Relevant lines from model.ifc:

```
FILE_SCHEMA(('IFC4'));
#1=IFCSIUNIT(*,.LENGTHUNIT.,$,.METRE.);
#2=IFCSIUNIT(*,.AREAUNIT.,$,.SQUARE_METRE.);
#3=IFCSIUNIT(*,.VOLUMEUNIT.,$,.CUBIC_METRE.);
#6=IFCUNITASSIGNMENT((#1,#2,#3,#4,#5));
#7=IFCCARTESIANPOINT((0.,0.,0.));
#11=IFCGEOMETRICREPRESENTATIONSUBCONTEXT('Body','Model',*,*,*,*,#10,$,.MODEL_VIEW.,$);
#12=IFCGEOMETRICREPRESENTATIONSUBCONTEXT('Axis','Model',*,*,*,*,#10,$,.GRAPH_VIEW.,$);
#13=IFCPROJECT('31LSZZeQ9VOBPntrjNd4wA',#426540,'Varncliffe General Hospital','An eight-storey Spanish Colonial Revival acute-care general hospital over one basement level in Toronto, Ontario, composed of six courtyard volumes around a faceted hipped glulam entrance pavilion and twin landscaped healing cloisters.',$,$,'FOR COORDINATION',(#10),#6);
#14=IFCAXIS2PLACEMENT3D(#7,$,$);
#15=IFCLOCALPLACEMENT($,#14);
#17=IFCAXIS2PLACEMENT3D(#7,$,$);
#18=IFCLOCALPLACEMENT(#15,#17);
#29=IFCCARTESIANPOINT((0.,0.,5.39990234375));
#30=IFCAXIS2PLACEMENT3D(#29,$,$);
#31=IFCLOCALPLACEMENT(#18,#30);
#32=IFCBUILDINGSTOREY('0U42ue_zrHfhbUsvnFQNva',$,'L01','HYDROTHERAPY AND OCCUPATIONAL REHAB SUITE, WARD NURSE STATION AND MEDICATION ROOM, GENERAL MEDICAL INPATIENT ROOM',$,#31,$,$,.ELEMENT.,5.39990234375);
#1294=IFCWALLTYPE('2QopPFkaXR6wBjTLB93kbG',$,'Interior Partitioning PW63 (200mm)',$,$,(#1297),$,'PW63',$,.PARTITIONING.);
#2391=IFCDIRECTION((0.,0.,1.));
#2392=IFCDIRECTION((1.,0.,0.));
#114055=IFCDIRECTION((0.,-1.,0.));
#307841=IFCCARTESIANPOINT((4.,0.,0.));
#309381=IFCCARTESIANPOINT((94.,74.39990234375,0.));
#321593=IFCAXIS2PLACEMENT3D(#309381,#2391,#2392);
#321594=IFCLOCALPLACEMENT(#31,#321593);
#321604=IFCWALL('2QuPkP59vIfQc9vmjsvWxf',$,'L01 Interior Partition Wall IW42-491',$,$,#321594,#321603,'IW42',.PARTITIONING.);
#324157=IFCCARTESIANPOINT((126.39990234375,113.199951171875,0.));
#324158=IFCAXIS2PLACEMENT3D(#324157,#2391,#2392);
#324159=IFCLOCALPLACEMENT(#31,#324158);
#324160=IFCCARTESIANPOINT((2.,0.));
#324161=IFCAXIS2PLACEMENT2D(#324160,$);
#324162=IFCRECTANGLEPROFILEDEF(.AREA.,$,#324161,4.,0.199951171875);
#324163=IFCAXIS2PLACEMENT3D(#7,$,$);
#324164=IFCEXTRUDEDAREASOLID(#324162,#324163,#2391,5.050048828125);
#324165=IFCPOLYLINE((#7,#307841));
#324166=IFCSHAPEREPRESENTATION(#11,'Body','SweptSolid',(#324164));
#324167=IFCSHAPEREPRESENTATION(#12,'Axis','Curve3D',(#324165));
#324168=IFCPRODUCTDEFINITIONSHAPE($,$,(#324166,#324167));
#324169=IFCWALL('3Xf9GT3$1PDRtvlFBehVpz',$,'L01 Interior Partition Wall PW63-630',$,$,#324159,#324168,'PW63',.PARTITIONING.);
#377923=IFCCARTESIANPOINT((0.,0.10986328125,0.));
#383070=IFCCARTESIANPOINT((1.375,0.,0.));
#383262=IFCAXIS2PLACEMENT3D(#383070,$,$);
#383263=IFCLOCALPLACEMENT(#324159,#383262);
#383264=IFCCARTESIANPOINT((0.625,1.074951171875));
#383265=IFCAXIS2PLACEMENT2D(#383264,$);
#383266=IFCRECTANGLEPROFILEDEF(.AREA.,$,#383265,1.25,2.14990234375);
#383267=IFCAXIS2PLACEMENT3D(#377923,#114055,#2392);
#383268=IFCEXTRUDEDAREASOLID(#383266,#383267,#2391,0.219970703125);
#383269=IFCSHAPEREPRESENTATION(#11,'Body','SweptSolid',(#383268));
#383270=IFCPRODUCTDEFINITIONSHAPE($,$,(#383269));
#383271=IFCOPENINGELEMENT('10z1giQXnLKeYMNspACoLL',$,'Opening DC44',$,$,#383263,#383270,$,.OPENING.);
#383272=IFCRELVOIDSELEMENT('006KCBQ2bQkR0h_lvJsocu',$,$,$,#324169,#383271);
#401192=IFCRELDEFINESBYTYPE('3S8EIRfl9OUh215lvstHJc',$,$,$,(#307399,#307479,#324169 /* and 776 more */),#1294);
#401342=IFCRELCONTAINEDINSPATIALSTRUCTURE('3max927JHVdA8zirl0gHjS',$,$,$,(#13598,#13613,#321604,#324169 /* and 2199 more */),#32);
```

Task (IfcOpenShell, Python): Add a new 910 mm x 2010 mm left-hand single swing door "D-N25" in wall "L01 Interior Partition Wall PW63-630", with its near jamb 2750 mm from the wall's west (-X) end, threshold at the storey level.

```python
import numpy as np
import ifcopenshell
import ifcopenshell.api.feature
import ifcopenshell.api.geometry
import ifcopenshell.api.root
import ifcopenshell.api.spatial
import ifcopenshell.geom
import ifcopenshell.util.element
import ifcopenshell.util.placement
import ifcopenshell.util.representation
import ifcopenshell.util.shape
import ifcopenshell.util.unit

model = ifcopenshell.open("model.ifc")
unit_scale = ifcopenshell.util.unit.calculate_unit_scale(model)
settings = ifcopenshell.geom.settings()


def volume(element):
    """Net volume in cubic metres, openings subtracted."""
    shape = ifcopenshell.geom.create_shape(settings, element)
    return ifcopenshell.util.shape.get_volume(shape.geometry)


wall = model.by_guid("3Xf9GT3$1PDRtvlFBehVpz")
storey = ifcopenshell.util.element.get_container(wall, ifc_class="IfcBuildingStorey")
context = ifcopenshell.util.representation.get_context(model, "Model", "Body", "MODEL_VIEW")
before = volume(wall)

width, height, from_end, sill = 0.91, 2.01, 2.75, 0.0  # metres

# The wall runs along its own X axis, and the end named is its -X end.
wall_shape = ifcopenshell.geom.create_shape(settings, wall)
x, y, z = ifcopenshell.util.shape.get_vertices(wall_shape.geometry).T
start = x.min() + from_end
face, thickness = float(y.min()), float(y.max() - y.min())
wall_matrix = ifcopenshell.util.placement.get_local_placement(wall.ObjectPlacement)
level = ifcopenshell.util.placement.get_local_placement(storey.ObjectPlacement)[2, 3]


def in_wall(x, y):
    """Placement at x, y metres in the wall's axes, at sill height."""
    matrix = wall_matrix.copy()
    matrix[:, 3] = wall_matrix @ np.array([x / unit_scale, y / unit_scale, 0.0, 1.0])
    matrix[2, 3] = level + sill / unit_scale
    return matrix


# Opening: a box that overshoots both wall faces by 50 mm.
opening = ifcopenshell.api.root.create_entity(model, ifc_class="IfcOpeningElement", predefined_type="OPENING")
box = ifcopenshell.api.geometry.add_wall_representation(
    model, context=context, length=width, height=height, thickness=thickness + 0.1
)
ifcopenshell.api.geometry.assign_representation(model, product=opening, representation=box)
ifcopenshell.api.geometry.edit_object_placement(model, product=opening, matrix=in_wall(start, face - 0.05), is_si=False)
ifcopenshell.api.feature.add_feature(model, feature=opening, element=wall)

door = ifcopenshell.api.root.create_entity(model, ifc_class="IfcDoor", name="D-N25", predefined_type="DOOR")
door.OverallWidth, door.OverallHeight = width / unit_scale, height / unit_scale
door.OperationType = "SINGLE_SWING_LEFT"
body = ifcopenshell.api.geometry.add_door_representation(
    model,
    context=context,
    overall_width=door.OverallWidth,
    overall_height=door.OverallHeight,
    operation_type="SINGLE_SWING_LEFT",
    lining_properties={"LiningDepth": thickness / unit_scale, "ThresholdDepth": thickness / unit_scale},
)
ifcopenshell.api.geometry.assign_representation(model, product=door, representation=body)
ifcopenshell.api.spatial.assign_container(model, products=[door], relating_structure=storey)
ifcopenshell.api.feature.add_filling(model, opening=opening, element=door)

# The lining spans the wall, so the door starts at the wall face.
ifcopenshell.api.geometry.edit_object_placement(model, product=door, matrix=in_wall(start, face), is_si=False)

after = volume(wall)

print(f"wall volume {before:.3f} -> {after:.3f} m3")

model.write("model-out.ifc")
```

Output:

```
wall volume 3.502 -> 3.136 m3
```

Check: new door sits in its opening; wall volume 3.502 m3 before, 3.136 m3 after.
